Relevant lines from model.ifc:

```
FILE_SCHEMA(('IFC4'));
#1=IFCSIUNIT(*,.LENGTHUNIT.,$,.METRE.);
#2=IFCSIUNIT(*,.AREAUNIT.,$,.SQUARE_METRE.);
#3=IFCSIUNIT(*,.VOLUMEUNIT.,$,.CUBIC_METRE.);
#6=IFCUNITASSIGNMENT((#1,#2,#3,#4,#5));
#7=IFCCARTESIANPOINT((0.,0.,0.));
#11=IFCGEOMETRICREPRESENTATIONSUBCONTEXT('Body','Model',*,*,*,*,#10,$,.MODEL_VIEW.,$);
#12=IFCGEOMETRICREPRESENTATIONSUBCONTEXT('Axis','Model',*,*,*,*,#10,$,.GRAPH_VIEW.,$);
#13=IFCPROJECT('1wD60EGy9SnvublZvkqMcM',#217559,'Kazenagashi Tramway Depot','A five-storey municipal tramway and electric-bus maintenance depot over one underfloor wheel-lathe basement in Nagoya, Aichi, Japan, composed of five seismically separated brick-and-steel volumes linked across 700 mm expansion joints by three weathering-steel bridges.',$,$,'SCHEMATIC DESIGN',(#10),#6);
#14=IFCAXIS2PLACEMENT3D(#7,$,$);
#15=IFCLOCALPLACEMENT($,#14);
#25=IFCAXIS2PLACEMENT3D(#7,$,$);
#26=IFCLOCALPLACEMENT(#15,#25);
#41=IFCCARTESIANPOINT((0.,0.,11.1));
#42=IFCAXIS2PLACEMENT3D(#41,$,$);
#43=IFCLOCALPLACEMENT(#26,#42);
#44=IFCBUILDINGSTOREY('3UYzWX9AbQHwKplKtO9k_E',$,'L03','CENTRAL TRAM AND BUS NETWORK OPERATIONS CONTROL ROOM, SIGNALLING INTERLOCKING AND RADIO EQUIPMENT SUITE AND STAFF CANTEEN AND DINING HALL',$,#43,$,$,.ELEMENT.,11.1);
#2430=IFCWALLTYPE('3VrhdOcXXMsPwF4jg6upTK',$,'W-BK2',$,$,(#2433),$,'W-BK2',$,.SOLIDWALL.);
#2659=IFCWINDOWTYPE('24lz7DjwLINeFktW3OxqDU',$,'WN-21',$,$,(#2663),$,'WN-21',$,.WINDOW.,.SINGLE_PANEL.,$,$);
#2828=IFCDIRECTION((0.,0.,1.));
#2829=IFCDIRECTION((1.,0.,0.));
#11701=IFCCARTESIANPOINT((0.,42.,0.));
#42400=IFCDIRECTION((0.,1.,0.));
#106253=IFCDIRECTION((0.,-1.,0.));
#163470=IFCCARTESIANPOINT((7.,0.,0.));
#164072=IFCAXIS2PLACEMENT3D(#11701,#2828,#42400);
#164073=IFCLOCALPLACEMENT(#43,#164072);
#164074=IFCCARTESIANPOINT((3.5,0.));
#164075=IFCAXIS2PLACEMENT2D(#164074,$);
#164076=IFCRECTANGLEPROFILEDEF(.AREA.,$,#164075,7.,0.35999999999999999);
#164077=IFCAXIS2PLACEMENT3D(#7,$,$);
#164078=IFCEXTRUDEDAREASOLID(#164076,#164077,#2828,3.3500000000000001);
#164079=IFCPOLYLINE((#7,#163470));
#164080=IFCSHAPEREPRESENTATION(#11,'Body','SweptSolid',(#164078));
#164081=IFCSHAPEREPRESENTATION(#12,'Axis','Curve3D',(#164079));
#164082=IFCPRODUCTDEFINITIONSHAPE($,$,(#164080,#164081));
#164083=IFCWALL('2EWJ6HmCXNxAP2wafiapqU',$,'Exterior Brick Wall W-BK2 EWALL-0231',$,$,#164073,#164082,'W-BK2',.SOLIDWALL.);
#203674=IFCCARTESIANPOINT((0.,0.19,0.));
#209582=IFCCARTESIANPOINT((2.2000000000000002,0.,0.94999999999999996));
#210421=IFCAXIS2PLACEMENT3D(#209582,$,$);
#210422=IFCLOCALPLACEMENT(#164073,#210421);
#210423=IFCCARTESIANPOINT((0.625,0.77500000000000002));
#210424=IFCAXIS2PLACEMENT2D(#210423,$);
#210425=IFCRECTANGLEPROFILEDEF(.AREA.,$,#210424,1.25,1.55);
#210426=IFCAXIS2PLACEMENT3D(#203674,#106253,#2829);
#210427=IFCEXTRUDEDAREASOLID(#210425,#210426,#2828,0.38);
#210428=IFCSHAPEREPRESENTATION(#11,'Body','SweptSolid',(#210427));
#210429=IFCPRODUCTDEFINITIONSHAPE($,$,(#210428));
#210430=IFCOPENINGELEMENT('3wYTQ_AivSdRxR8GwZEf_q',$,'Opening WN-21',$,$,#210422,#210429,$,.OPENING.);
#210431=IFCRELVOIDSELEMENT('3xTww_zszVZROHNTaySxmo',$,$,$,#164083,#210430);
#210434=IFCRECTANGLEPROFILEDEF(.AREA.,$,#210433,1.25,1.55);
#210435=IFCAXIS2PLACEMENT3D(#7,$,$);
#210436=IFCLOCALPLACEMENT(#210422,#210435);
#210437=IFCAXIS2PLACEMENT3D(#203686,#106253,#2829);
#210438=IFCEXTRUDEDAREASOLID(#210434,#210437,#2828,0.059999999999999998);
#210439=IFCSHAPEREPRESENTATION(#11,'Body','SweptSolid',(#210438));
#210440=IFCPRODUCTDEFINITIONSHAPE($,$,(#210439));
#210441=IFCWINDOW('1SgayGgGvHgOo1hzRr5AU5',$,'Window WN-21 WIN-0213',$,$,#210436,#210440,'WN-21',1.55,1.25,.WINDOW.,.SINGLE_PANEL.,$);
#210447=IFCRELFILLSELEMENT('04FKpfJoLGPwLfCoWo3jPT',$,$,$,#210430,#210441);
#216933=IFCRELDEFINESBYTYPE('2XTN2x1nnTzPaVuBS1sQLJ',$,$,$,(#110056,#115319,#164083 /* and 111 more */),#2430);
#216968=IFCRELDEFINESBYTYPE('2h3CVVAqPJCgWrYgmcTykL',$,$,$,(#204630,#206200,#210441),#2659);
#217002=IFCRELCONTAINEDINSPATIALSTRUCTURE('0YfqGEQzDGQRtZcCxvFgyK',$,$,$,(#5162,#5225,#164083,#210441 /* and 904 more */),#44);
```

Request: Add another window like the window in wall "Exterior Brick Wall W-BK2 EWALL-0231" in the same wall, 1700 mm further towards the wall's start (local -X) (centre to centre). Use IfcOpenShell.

```python
import ifcopenshell
import ifcopenshell.api.feature
import ifcopenshell.api.geometry
import ifcopenshell.api.root
import ifcopenshell.geom
import ifcopenshell.util.element
import ifcopenshell.util.placement
import ifcopenshell.util.shape
import ifcopenshell.util.unit

model = ifcopenshell.open("model.ifc")
unit_scale = ifcopenshell.util.unit.calculate_unit_scale(model)
settings = ifcopenshell.geom.settings()


def volume(element):
    """Net volume in cubic metres, openings subtracted."""
    shape = ifcopenshell.geom.create_shape(settings, element)
    return ifcopenshell.util.shape.get_volume(shape.geometry)


window = model.by_id(210441)
opening = window.FillsVoids[0].RelatingOpeningElement
wall = opening.VoidsElements[0].RelatingBuildingElement
before = volume(wall)
shift = ifcopenshell.util.placement.get_local_placement(wall.ObjectPlacement)[:3, 0] * -1.7 / unit_scale

# copy_class copies the void relationship, type, container and properties, but no geometry.
new_opening = ifcopenshell.api.root.copy_class(model, product=opening)
new_opening.Representation = ifcopenshell.util.element.copy_deep(
    model, opening.Representation, exclude=["IfcGeometricRepresentationContext", "IfcRepresentationMap"]
)
new_window = ifcopenshell.api.root.copy_class(model, product=window)
new_window.Representation = ifcopenshell.util.element.copy_deep(
    model, window.Representation, exclude=["IfcGeometricRepresentationContext", "IfcRepresentationMap"]
)
new_window.Tag = None
ifcopenshell.api.feature.add_filling(model, opening=new_opening, element=new_window)

for old, new in ((opening, new_opening), (window, new_window)):
    matrix = ifcopenshell.util.placement.get_local_placement(old.ObjectPlacement)
    matrix[:3, 3] += shift
    ifcopenshell.api.geometry.edit_object_placement(model, product=new, matrix=matrix, is_si=False)

after = volume(wall)

print(f"wall volume {before:.3f} -> {after:.3f} m3")

model.write("model_rev.ifc")
```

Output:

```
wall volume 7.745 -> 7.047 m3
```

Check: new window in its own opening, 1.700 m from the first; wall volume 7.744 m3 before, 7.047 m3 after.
